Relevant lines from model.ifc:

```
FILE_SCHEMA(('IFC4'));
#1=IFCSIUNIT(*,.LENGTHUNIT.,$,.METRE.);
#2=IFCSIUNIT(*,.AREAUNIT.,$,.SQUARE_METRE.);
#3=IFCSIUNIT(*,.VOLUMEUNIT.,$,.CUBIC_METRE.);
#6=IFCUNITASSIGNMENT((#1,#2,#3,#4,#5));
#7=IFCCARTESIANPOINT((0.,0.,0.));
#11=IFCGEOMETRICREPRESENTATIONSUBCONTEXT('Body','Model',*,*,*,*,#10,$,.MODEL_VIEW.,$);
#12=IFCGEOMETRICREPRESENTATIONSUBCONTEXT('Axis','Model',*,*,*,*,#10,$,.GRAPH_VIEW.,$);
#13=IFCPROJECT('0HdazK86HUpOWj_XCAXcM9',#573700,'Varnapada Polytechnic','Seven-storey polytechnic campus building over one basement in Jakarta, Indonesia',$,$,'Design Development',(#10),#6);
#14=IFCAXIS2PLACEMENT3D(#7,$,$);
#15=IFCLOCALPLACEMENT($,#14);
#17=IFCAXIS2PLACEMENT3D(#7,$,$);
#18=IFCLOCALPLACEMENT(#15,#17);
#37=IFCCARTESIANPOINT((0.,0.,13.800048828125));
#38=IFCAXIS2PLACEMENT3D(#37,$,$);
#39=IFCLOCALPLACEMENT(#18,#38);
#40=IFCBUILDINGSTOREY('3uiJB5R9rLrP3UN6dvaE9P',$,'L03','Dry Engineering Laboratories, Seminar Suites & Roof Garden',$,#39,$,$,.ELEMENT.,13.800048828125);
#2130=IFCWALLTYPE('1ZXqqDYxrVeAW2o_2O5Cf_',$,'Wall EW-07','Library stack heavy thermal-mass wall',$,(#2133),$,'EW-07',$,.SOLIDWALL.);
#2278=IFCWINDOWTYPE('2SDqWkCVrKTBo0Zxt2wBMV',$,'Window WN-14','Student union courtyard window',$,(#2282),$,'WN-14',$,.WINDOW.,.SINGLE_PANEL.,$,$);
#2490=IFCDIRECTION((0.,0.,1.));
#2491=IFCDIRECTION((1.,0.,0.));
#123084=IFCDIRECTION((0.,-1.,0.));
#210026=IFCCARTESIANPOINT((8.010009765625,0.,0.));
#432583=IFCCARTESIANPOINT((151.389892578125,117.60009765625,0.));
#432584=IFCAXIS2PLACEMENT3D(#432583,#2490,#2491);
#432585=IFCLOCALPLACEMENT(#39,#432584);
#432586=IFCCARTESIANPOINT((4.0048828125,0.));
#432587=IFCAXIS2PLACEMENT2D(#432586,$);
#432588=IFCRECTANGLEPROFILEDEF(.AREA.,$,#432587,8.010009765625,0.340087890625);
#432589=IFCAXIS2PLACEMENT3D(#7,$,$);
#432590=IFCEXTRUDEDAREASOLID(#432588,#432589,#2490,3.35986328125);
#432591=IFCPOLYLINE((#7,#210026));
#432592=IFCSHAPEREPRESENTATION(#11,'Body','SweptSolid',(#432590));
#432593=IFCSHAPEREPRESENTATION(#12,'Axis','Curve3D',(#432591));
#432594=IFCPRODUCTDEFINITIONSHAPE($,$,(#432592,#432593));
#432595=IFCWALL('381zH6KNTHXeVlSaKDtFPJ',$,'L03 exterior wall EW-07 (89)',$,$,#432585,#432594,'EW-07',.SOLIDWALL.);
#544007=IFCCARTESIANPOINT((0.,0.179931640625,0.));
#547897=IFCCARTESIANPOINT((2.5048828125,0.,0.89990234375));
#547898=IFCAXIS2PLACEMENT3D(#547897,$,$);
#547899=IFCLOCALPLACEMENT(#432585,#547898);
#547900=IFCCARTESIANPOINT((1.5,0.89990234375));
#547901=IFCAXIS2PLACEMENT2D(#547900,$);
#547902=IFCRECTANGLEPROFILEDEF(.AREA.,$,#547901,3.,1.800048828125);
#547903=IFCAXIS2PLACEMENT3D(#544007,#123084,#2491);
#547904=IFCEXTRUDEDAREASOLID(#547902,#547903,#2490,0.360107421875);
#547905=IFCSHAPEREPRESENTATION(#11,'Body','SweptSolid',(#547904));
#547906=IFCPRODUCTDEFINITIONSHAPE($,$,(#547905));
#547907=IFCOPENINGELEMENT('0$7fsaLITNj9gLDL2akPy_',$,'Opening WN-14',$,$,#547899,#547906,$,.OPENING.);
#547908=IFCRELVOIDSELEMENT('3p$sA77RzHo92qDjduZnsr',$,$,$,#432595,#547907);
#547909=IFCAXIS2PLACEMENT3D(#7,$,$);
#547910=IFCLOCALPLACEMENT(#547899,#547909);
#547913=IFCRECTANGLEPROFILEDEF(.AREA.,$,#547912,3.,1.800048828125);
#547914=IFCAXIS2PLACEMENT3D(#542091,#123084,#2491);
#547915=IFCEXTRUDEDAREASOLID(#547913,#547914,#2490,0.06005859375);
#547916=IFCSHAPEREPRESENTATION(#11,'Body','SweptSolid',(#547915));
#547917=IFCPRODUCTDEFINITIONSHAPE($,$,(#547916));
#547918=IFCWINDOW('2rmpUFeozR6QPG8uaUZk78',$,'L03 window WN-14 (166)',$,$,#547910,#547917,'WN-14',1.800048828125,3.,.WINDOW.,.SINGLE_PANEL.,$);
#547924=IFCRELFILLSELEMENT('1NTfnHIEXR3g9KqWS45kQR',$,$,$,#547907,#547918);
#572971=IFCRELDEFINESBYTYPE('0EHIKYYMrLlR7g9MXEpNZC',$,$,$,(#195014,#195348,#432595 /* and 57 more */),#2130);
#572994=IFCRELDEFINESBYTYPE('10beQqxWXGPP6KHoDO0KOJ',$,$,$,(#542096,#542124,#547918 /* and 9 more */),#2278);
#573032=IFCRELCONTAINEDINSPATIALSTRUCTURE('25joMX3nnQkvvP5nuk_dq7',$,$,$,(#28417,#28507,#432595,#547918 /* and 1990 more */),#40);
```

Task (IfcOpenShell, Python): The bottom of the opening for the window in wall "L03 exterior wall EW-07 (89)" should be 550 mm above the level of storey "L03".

```python
import numpy as np
import ifcopenshell
import ifcopenshell.api.geometry
import ifcopenshell.geom
import ifcopenshell.util.element
import ifcopenshell.util.placement
import ifcopenshell.util.shape
import ifcopenshell.util.unit

model = ifcopenshell.open("model.ifc")
unit_scale = ifcopenshell.util.unit.calculate_unit_scale(model)

window = model.by_id(547918)
opening = window.FillsVoids[0].RelatingOpeningElement
storey = ifcopenshell.util.element.get_container(window, ifc_class="IfcBuildingStorey")
level = ifcopenshell.util.placement.get_local_placement(storey.ObjectPlacement)[2, 3]

# The opening's origin need not be at the sill, so measure its lowest point.
shape = ifcopenshell.geom.create_shape(ifcopenshell.geom.settings(), opening)
bottom = ifcopenshell.util.shape.get_shape_bottom_elevation(shape, shape.geometry) / unit_scale
dz = level + 0.55 - bottom

shift = np.array([0.0, 0.0, dz])
# The window is placed relative to its opening, so it follows when the opening moves.
matrix = ifcopenshell.util.placement.get_local_placement(opening.ObjectPlacement)
matrix[:3, 3] += shift
ifcopenshell.api.geometry.edit_object_placement(
    model, product=opening, matrix=matrix, is_si=False, should_transform_children=True
)

print(f"moved by {dz * unit_scale:+.3f} m")

model.write("model_rev.ifc")
```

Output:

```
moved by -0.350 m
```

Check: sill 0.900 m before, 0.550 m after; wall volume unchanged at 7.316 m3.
